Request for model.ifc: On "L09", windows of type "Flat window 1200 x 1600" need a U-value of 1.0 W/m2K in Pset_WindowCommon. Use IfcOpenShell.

First a look at what the model holds.

```python
import ifcopenshell
import ifcopenshell.util.element

model = ifcopenshell.open("model.ifc")
print(model.schema)
storey = next(s for s in model.by_type("IfcBuildingStorey") if s.Name == "L09")
windows = [e for e in ifcopenshell.util.element.get_decomposition(storey) if e.is_a("IfcWindow")]
seen = {}
for e in windows:
    element_type = ifcopenshell.util.element.get_type(e)
    key = (element_type.Name if element_type != e and element_type else None, ifcopenshell.util.element.get_pset(e, "Pset_WindowCommon", "ThermalTransmittance"))
    seen[key] = seen.get(key, 0) + 1
for (name, value), count in sorted(seen.items(), key=str):
    print(count, "x", name, "|", value)
```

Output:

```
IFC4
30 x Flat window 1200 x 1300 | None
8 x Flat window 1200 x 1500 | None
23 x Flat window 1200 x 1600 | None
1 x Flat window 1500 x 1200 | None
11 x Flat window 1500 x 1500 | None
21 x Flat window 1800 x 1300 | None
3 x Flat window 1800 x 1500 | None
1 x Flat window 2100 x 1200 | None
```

```python
import ifcopenshell
import ifcopenshell.api.pset
import ifcopenshell.util.element

model = ifcopenshell.open("model.ifc")

storey = next(s for s in model.by_type("IfcBuildingStorey") if s.Name == "L09")
windows = [e for e in ifcopenshell.util.element.get_decomposition(storey) if e.is_a("IfcWindow")]

count = 0
for e in windows:
    element_type = ifcopenshell.util.element.get_type(e)
    if element_type in (None, e) or element_type.Name != "Flat window 1200 x 1600":
        continue
    # add_pset returns the element's existing set when there is one.
    pset = ifcopenshell.api.pset.add_pset(model, product=e, name="Pset_WindowCommon")
    ifcopenshell.api.pset.edit_pset(model, pset=pset, properties={"ThermalTransmittance": 1.0})
    count += 1

print(count, "windows updated")

model.write("model_edited.ifc")
```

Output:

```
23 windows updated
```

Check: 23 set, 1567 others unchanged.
